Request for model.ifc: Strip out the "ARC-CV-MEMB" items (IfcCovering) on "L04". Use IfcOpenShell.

First a look at what the model holds.

```python
import ifcopenshell
import ifcopenshell.util.element

model = ifcopenshell.open("model.ifc")
print(model.schema)
storey = next(s for s in model.by_type("IfcBuildingStorey") if s.Name == "L04")
coverings = [e for e in ifcopenshell.util.element.get_decomposition(storey) if e.is_a("IfcCovering")]
seen = {}
for e in coverings:
    element_type = ifcopenshell.util.element.get_type(e)
    name = element_type.Name if element_type not in (None, e) else None
    seen[name] = seen.get(name, 0) + 1
for name, count in sorted(seen.items(), key=str):
    print(count, "x", name)
```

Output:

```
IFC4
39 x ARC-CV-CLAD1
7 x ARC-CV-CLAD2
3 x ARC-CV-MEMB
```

```python
import ifcopenshell
import ifcopenshell.api.root
import ifcopenshell.util.element

model = ifcopenshell.open("model.ifc")

storey = next(s for s in model.by_type("IfcBuildingStorey") if s.Name == "L04")
coverings = [e for e in ifcopenshell.util.element.get_decomposition(storey) if e.is_a("IfcCovering")]
targets = [e for e in coverings if (t := ifcopenshell.util.element.get_type(e)) not in (None, e) and t.Name == "ARC-CV-MEMB"]

for e in targets:
    ifcopenshell.api.root.remove_product(model, product=e)
print(len(targets), "removed")

model.write("model_updated.ifc")
```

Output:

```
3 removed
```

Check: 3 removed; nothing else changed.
